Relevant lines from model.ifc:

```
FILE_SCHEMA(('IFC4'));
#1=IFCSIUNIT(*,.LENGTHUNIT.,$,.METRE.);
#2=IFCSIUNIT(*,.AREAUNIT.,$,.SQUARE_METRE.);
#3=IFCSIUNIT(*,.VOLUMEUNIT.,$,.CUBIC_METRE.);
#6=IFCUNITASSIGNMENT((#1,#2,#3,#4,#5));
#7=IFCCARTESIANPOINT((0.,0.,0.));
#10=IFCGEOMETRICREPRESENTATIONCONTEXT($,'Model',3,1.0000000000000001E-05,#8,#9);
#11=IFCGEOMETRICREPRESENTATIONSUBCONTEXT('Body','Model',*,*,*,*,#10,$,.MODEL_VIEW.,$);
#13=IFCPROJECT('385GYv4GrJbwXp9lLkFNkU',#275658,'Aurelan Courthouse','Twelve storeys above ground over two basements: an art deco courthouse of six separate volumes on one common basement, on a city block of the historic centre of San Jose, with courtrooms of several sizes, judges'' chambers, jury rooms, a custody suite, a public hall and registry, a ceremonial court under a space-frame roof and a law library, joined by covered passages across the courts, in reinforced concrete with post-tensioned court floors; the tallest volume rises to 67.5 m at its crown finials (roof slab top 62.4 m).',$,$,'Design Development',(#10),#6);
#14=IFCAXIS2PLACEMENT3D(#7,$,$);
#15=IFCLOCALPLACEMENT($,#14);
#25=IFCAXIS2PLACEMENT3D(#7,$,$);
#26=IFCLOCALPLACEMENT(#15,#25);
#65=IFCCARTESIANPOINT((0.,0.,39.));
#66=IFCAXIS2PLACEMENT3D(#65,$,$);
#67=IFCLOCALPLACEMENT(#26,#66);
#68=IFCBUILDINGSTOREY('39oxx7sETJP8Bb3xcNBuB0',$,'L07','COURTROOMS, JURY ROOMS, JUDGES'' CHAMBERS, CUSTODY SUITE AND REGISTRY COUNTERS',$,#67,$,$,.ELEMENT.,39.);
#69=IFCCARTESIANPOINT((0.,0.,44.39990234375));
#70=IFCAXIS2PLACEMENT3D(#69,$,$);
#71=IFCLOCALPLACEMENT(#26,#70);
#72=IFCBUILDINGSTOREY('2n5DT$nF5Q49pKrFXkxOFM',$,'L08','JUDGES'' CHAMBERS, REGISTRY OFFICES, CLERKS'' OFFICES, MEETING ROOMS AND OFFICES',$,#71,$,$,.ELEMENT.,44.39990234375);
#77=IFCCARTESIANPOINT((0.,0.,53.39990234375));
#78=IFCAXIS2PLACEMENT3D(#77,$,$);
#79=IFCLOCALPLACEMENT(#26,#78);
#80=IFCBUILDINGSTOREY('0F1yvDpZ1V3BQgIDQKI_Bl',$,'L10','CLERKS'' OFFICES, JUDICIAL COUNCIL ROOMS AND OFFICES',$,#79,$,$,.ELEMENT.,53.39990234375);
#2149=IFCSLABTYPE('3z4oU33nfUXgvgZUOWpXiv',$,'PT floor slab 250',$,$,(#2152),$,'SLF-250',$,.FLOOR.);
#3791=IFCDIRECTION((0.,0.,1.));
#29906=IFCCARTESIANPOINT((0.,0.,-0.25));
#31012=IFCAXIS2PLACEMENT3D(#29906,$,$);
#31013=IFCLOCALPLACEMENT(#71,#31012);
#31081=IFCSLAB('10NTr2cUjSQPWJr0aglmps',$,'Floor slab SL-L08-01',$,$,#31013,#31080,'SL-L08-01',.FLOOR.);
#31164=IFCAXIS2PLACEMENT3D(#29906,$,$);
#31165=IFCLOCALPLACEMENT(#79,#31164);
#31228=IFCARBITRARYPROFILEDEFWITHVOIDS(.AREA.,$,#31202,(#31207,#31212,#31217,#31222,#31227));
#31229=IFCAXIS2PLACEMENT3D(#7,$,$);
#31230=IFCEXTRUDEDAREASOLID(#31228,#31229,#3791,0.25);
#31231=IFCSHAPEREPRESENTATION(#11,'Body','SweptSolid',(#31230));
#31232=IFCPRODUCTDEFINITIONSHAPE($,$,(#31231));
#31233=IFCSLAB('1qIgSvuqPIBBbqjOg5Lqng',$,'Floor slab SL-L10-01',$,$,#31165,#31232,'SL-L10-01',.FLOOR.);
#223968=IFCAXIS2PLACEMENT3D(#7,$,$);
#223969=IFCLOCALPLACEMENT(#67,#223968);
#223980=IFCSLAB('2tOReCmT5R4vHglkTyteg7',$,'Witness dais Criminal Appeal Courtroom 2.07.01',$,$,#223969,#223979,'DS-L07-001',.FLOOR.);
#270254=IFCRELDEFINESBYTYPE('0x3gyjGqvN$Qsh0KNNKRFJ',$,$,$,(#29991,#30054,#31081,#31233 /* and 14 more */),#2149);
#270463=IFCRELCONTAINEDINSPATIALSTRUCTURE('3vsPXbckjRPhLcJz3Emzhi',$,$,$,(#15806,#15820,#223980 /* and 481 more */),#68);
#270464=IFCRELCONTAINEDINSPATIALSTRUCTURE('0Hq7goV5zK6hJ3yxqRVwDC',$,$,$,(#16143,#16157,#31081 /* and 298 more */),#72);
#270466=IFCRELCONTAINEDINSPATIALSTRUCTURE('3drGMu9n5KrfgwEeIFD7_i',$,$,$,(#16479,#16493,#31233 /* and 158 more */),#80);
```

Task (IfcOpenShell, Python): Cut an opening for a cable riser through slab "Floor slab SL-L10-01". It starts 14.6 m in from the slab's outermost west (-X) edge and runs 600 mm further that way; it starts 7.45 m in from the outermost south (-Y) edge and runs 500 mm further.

```python
import numpy as np
import ifcopenshell
import ifcopenshell.api.feature
import ifcopenshell.api.geometry
import ifcopenshell.api.root
import ifcopenshell.geom
import ifcopenshell.util.placement
import ifcopenshell.util.representation
import ifcopenshell.util.shape
import ifcopenshell.util.unit

model = ifcopenshell.open("model.ifc")
unit_scale = ifcopenshell.util.unit.calculate_unit_scale(model)
settings = ifcopenshell.geom.settings()


def volume(element):
    """Net volume in cubic metres, openings subtracted."""
    shape = ifcopenshell.geom.create_shape(settings, element)
    return ifcopenshell.util.shape.get_volume(shape.geometry)


slab = model.by_guid("1qIgSvuqPIBBbqjOg5Lqng")
before = volume(slab)

# Extent in the slab's own axes, in metres. The edges named are its -X and -Y sides.
slab_shape = ifcopenshell.geom.create_shape(settings, slab)
vertices = ifcopenshell.util.shape.get_vertices(slab_shape.geometry)
x_min, y_min, bottom = vertices.min(axis=0)
top = vertices[:, 2].max()

opening = ifcopenshell.api.root.create_entity(model, ifc_class="IfcOpeningElement", name="Cable riser opening", predefined_type="OPENING")
context = ifcopenshell.util.representation.get_context(model, "Model", "Body", "MODEL_VIEW")
width, depth = 0.6, 0.5
outline = [(0.0, 0.0), (width, 0.0), (width, depth), (0.0, depth), (0.0, 0.0)]
# Overshoot both faces by 50 mm so the cut is clean.
shape = ifcopenshell.api.geometry.add_slab_representation(
    model, context=context, depth=top - bottom + 0.1, polyline=outline
)
ifcopenshell.api.geometry.assign_representation(model, product=opening, representation=shape)

matrix = ifcopenshell.util.placement.get_local_placement(slab.ObjectPlacement)
matrix[:, 3] = matrix @ np.append(np.array([x_min + 14.6, y_min + 7.45, bottom - 0.05]) / unit_scale, 1.0)
ifcopenshell.api.geometry.edit_object_placement(model, product=opening, matrix=matrix, is_si=False)
ifcopenshell.api.feature.add_feature(model, feature=opening, element=slab)

after = volume(slab)

print(f"slab volume {before:.3f} -> {after:.3f} m3")

model.write("model_updated.ifc")
```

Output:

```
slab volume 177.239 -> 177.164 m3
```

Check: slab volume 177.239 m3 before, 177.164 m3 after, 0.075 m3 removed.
